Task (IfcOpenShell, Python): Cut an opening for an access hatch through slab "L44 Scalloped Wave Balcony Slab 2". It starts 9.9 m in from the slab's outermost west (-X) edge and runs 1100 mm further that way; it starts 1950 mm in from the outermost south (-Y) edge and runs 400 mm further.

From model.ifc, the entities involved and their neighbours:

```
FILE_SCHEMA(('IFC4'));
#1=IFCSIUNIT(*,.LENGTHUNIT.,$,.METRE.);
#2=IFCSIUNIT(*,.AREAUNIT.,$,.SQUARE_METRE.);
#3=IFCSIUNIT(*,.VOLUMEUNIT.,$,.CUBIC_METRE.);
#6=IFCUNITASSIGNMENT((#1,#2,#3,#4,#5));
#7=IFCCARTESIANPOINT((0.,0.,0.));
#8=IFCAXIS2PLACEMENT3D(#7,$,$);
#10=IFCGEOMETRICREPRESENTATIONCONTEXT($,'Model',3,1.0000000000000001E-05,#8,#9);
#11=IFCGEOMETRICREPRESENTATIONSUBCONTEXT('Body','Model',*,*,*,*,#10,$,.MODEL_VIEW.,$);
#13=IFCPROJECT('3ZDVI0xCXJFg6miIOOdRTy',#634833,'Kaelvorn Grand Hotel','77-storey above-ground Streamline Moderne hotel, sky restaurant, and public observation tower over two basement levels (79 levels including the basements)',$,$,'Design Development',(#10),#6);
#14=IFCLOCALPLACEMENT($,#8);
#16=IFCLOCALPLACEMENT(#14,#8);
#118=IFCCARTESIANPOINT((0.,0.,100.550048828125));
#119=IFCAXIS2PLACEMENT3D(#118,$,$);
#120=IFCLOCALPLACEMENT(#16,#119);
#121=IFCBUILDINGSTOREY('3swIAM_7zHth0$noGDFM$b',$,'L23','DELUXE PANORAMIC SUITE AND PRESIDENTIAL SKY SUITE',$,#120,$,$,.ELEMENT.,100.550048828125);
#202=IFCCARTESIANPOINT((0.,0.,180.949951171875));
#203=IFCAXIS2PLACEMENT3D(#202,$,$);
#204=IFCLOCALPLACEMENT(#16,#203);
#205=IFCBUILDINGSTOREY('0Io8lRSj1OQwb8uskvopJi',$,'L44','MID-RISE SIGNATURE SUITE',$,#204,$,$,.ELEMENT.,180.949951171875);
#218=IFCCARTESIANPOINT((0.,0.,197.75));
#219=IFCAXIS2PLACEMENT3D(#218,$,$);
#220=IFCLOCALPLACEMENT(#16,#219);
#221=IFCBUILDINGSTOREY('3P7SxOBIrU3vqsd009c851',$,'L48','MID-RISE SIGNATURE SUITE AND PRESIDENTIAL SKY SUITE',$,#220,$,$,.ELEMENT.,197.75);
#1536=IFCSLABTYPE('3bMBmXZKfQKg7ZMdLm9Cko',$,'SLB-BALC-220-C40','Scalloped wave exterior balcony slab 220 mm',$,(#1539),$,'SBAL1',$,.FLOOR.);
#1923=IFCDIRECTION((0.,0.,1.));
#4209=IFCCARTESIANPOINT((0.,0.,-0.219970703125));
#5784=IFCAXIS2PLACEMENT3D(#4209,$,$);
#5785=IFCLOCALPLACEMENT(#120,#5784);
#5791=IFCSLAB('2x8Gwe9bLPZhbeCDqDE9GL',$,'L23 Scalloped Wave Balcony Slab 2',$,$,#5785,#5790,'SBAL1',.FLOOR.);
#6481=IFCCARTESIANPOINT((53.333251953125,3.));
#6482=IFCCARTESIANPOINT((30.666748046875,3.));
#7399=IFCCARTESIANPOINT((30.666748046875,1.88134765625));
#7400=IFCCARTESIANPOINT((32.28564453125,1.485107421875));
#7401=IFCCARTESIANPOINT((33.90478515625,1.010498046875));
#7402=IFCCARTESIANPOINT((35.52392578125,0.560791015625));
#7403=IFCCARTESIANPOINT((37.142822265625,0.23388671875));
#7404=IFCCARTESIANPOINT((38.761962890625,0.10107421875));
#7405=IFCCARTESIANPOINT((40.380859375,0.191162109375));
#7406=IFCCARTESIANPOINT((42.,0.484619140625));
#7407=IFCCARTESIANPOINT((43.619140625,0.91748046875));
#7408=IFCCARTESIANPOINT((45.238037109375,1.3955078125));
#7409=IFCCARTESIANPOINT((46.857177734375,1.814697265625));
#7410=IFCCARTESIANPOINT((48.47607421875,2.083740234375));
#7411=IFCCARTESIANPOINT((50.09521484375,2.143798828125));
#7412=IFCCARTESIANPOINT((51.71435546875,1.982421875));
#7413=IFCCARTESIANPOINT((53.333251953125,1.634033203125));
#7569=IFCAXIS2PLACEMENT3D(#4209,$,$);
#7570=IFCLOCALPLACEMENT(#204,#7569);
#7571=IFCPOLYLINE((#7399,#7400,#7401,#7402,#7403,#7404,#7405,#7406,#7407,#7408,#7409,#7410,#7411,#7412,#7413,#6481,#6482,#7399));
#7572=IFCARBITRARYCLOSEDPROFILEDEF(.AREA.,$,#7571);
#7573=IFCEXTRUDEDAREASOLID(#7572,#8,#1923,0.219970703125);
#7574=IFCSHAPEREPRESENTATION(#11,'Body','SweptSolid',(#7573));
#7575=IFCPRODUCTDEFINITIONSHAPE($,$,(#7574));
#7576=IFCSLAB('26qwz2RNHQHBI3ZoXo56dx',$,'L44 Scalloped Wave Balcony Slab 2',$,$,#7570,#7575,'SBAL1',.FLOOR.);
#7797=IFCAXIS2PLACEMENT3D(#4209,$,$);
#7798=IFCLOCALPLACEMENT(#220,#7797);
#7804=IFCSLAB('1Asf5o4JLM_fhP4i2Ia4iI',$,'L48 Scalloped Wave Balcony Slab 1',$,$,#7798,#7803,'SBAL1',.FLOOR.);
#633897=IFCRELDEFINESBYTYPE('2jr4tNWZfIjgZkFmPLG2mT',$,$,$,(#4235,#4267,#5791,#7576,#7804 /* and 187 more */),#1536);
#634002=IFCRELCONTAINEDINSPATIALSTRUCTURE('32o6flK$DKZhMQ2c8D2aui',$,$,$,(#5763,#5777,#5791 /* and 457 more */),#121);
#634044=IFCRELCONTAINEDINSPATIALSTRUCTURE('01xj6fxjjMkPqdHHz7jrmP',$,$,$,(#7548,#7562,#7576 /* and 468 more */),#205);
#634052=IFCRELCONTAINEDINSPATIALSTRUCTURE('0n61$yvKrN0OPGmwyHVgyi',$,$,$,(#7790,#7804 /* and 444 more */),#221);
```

```python
import numpy as np
import ifcopenshell
import ifcopenshell.api.feature
import ifcopenshell.api.geometry
import ifcopenshell.api.root
import ifcopenshell.geom
import ifcopenshell.util.placement
import ifcopenshell.util.representation
import ifcopenshell.util.shape
import ifcopenshell.util.unit

model = ifcopenshell.open("model.ifc")
unit_scale = ifcopenshell.util.unit.calculate_unit_scale(model)
settings = ifcopenshell.geom.settings()


def volume(element):
    """Net volume in cubic metres, openings subtracted."""
    shape = ifcopenshell.geom.create_shape(settings, element)
    return ifcopenshell.util.shape.get_volume(shape.geometry)


slab = model.by_id(7576)
before = volume(slab)

# Extent in the slab's own axes, in metres. The edges named are its -X and -Y sides.
slab_shape = ifcopenshell.geom.create_shape(settings, slab)
vertices = ifcopenshell.util.shape.get_vertices(slab_shape.geometry)
x_min, y_min, bottom = vertices.min(axis=0)
top = vertices[:, 2].max()

opening = ifcopenshell.api.root.create_entity(model, ifc_class="IfcOpeningElement", name="Access hatch opening", predefined_type="OPENING")
context = ifcopenshell.util.representation.get_context(model, "Model", "Body", "MODEL_VIEW")
width, depth = 1.1, 0.4
outline = [(0.0, 0.0), (width, 0.0), (width, depth), (0.0, depth), (0.0, 0.0)]
# Overshoot both faces by 50 mm so the cut is clean.
shape = ifcopenshell.api.geometry.add_slab_representation(
    model, context=context, depth=top - bottom + 0.1, polyline=outline
)
ifcopenshell.api.geometry.assign_representation(model, product=opening, representation=shape)

matrix = ifcopenshell.util.placement.get_local_placement(slab.ObjectPlacement)
matrix[:, 3] = matrix @ np.append(np.array([x_min + 9.9, y_min + 1.95, bottom - 0.05]) / unit_scale, 1.0)
ifcopenshell.api.geometry.edit_object_placement(model, product=opening, matrix=matrix, is_si=False)
ifcopenshell.api.feature.add_feature(model, feature=opening, element=slab)

after = volume(slab)

print(f"slab volume {before:.3f} -> {after:.3f} m3")

model.write("model-out.ifc")
```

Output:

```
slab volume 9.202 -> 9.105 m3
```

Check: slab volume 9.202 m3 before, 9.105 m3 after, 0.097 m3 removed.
